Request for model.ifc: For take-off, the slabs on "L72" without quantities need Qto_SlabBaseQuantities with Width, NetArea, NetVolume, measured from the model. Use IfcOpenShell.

First a look at what the model holds.

```python
import ifcopenshell
import ifcopenshell.util.element
import ifcopenshell.util.unit

model = ifcopenshell.open("model.ifc")
print(model.schema)
for unit_type in ("LENGTHUNIT", "AREAUNIT", "VOLUMEUNIT"):
    print(unit_type, ifcopenshell.util.unit.calculate_unit_scale(model, unit_type))
storey = next(s for s in model.by_type("IfcBuildingStorey") if s.Name == "L72")
slabs = [e for e in ifcopenshell.util.element.get_decomposition(storey) if e.is_a("IfcSlab")]
for e in sorted(slabs, key=lambda e: e.id()):
    print(e.id(), e.is_a(), e.Name, list(ifcopenshell.util.element.get_psets(e, qtos_only=True)), sep=" | ")
```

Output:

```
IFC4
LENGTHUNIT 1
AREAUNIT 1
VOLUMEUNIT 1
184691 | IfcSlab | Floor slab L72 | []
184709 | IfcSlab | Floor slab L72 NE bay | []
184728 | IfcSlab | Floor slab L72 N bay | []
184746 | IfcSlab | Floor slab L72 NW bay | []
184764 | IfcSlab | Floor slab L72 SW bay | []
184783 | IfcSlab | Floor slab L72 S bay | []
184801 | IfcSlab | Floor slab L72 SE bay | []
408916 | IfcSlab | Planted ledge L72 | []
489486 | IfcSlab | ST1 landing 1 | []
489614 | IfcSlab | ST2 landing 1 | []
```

```python
import ifcopenshell
import ifcopenshell.api.pset
import ifcopenshell.geom
import ifcopenshell.util.element
import ifcopenshell.util.shape
import ifcopenshell.util.unit

model = ifcopenshell.open("model.ifc")
unit_scale = ifcopenshell.util.unit.calculate_unit_scale(model)
area_scale = ifcopenshell.util.unit.calculate_unit_scale(model, "AREAUNIT")
volume_scale = ifcopenshell.util.unit.calculate_unit_scale(model, "VOLUMEUNIT")
settings = ifcopenshell.geom.settings()

storey = next(s for s in model.by_type("IfcBuildingStorey") if s.Name == "L72")
slabs = [e for e in ifcopenshell.util.element.get_decomposition(storey) if e.is_a("IfcSlab")]

for e in sorted(slabs, key=lambda e: e.id()):
    if ifcopenshell.util.element.get_psets(e, qtos_only=True, should_inherit=False):
        continue
    # Geometry comes back in metres, in the element's own axes.
    shape = ifcopenshell.geom.create_shape(settings, e)
    values = {
        "Width": ifcopenshell.util.shape.get_z(shape.geometry) / unit_scale,
        "NetArea": ifcopenshell.util.shape.get_footprint_area(shape.geometry) / area_scale,
        "NetVolume": ifcopenshell.util.shape.get_volume(shape.geometry) / volume_scale,
    }
    qto = ifcopenshell.api.pset.add_qto(model, product=e, name="Qto_SlabBaseQuantities")
    ifcopenshell.api.pset.edit_qto(model, qto=qto, properties=values)
    print(e.id(), {k: round(v, 3) for k, v in values.items()})

model.write("model-out.ifc")
```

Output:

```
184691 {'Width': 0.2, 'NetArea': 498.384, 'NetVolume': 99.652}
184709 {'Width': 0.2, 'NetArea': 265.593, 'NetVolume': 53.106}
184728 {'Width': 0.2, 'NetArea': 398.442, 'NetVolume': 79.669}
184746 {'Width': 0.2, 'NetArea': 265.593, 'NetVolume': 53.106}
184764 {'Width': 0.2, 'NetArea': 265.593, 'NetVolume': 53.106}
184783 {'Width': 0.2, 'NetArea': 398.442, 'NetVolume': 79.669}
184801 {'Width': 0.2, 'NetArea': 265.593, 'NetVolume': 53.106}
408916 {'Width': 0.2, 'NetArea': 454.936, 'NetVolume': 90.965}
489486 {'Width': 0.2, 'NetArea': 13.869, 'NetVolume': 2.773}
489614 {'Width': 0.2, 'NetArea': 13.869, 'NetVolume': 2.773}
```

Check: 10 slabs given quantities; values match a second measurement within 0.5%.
